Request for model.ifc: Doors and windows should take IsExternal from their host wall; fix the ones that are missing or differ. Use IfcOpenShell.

First a look at what the model holds.

```python
import ifcopenshell
import ifcopenshell.util.element

model = ifcopenshell.open("model.ifc")
print(model.schema)
seen = {}
for e in model.by_type("IfcDoor") + model.by_type("IfcWindow"):
    if not e.FillsVoids:
        continue
    host = e.FillsVoids[0].RelatingOpeningElement.VoidsElements[0].RelatingBuildingElement
    own = ifcopenshell.util.element.get_pset(e, f"Pset_{e.is_a()[3:].removesuffix('StandardCase')}Common", "IsExternal")
    wall = ifcopenshell.util.element.get_pset(host, "Pset_WallCommon", "IsExternal")
    seen[e.is_a(), own, wall] = seen.get((e.is_a(), own, wall), 0) + 1
for (cls, own, wall), count in sorted(seen.items(), key=str):
    print(count, cls, "IsExternal:", own, "| host wall:", wall)
```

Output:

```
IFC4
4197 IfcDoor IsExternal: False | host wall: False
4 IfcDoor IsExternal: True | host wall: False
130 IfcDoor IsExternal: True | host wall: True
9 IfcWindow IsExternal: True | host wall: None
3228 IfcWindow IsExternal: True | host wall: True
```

```python
import ifcopenshell
import ifcopenshell.api.pset
import ifcopenshell.util.element

model = ifcopenshell.open("model.ifc")

count = 0
for ifc_class, pset_name in (("IfcDoor", "Pset_DoorCommon"), ("IfcWindow", "Pset_WindowCommon")):
    for e in model.by_type(ifc_class):
        if not e.FillsVoids:
            continue
        host = e.FillsVoids[0].RelatingOpeningElement.VoidsElements[0].RelatingBuildingElement
        external = ifcopenshell.util.element.get_pset(host, "Pset_WallCommon", "IsExternal")
        if external is None or ifcopenshell.util.element.get_pset(e, pset_name, "IsExternal") == external:
            continue
        pset = ifcopenshell.api.pset.add_pset(model, product=e, name=pset_name)
        ifcopenshell.api.pset.edit_pset(model, pset=pset, properties={"IsExternal": external})
        count += 1

print(count, "updated")

model.write("model_updated.ifc")
```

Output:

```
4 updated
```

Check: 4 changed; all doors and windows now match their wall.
